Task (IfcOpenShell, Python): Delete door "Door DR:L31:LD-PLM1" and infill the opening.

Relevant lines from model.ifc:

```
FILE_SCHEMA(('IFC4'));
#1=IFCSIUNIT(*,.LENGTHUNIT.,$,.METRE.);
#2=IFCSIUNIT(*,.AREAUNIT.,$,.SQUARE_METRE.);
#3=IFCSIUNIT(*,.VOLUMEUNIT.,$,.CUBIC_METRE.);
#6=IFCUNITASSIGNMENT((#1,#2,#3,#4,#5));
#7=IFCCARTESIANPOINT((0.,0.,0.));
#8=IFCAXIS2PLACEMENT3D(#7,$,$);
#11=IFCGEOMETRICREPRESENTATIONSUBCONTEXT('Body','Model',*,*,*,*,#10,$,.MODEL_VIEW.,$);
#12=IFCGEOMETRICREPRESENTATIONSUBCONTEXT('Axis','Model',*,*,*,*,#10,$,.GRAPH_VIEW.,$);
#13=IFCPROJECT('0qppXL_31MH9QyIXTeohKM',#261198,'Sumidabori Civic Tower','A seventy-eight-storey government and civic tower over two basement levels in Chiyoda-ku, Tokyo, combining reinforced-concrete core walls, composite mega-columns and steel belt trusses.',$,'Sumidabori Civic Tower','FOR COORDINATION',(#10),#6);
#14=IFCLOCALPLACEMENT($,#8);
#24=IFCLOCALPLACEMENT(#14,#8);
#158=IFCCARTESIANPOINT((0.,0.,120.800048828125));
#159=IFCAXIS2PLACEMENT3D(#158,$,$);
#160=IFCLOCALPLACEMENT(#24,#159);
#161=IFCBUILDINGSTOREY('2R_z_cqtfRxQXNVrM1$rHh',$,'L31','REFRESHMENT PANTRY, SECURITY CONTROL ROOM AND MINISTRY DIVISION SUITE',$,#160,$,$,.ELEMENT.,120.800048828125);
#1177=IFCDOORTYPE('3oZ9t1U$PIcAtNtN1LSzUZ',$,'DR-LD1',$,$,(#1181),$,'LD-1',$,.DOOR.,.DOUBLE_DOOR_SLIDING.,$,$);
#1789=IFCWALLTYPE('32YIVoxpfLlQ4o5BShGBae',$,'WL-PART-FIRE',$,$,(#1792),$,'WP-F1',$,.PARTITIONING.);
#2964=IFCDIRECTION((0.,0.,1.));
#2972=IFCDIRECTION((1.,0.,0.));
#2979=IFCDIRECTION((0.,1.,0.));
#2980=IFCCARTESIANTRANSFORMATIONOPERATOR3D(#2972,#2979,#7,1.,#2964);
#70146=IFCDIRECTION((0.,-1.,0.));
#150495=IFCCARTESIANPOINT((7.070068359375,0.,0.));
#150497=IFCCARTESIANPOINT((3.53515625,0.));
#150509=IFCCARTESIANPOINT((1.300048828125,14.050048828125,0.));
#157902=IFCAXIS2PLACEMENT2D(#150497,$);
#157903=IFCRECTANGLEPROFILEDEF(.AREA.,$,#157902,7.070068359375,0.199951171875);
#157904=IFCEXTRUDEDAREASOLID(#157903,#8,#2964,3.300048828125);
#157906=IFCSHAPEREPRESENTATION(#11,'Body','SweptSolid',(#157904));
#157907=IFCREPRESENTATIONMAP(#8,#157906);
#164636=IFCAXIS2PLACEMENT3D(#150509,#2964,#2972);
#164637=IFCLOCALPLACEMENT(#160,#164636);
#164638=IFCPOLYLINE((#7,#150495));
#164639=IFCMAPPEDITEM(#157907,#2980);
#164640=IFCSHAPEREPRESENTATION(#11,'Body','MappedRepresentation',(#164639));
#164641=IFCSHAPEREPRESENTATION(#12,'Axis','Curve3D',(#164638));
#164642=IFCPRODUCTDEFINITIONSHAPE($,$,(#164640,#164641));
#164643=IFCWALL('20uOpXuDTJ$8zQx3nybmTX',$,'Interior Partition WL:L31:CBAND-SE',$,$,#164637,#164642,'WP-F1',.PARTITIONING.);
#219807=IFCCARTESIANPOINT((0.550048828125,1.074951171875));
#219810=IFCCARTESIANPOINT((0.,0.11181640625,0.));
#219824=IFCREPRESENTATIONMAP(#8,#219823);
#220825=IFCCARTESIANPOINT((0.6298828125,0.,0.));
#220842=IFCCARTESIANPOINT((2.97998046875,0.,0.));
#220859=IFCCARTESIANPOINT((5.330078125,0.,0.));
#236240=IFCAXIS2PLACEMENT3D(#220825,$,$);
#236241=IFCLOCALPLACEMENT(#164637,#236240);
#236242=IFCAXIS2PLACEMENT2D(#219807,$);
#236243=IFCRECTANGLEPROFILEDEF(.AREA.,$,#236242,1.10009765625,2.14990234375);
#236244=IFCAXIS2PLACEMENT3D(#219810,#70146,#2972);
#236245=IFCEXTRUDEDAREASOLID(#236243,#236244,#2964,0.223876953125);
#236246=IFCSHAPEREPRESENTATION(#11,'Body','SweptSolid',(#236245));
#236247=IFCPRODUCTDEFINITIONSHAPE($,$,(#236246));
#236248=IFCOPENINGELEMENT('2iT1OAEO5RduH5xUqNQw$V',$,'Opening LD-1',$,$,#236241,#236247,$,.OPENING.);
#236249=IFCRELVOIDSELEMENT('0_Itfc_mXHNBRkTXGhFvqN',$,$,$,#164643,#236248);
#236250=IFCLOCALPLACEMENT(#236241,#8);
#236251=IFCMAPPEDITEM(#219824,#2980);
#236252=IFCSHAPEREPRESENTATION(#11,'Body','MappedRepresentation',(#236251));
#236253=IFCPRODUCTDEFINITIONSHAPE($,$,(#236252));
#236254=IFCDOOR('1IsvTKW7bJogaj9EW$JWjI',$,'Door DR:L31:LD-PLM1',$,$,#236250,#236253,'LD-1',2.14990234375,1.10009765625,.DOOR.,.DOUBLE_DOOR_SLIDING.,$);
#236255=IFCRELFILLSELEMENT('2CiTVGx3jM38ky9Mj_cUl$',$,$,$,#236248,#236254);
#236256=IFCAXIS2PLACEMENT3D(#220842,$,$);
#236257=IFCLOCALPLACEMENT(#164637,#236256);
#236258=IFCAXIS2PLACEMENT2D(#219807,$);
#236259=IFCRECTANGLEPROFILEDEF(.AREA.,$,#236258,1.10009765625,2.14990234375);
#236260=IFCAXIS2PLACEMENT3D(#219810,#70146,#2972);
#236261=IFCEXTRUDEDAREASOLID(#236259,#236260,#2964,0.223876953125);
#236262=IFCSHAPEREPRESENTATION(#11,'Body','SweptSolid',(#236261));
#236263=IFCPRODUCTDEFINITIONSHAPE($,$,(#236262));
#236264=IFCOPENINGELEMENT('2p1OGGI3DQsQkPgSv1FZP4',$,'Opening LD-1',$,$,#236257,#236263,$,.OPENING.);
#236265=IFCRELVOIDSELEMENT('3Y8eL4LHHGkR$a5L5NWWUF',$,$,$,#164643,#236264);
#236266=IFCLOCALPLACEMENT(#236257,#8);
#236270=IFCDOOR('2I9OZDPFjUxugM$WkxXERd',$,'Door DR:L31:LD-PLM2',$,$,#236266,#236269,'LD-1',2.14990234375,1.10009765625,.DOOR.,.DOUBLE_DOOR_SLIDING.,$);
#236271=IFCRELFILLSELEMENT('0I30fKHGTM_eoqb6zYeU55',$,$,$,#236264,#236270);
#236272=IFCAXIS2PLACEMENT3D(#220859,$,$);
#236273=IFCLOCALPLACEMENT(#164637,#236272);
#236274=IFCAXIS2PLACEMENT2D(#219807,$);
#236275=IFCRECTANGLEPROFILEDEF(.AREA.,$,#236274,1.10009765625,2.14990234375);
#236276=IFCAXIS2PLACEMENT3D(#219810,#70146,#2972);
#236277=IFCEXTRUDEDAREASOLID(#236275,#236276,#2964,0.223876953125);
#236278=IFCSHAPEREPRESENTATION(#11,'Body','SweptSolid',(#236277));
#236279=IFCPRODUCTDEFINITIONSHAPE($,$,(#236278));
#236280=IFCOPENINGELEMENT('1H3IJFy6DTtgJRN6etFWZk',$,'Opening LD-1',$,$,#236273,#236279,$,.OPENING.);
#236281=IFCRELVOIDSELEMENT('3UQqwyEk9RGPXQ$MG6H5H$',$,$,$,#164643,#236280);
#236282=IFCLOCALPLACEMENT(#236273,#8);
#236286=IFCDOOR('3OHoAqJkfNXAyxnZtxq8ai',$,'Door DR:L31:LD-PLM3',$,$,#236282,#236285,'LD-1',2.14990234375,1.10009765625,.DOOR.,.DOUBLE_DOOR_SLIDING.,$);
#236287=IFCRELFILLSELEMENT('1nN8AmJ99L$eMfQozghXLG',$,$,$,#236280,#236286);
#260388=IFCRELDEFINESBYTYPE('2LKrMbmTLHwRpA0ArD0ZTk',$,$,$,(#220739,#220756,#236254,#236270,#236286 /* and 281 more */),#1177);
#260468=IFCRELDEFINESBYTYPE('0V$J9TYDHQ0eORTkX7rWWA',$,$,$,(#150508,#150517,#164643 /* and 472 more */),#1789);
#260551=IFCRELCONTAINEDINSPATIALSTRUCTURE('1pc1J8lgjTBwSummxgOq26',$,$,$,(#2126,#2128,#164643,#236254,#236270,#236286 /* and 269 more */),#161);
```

```python
import ifcopenshell
import ifcopenshell.api.feature
import ifcopenshell.api.root
import ifcopenshell.geom
import ifcopenshell.util.shape

model = ifcopenshell.open("model.ifc")
settings = ifcopenshell.geom.settings()


def volume(element):
    """Net volume in cubic metres, openings subtracted."""
    shape = ifcopenshell.geom.create_shape(settings, element)
    return ifcopenshell.util.shape.get_volume(shape.geometry)


door = model.by_id(236254)
opening = door.FillsVoids[0].RelatingOpeningElement
wall = opening.VoidsElements[0].RelatingBuildingElement
before = volume(wall)

ifcopenshell.api.root.remove_product(model, product=door)
ifcopenshell.api.feature.remove_feature(model, feature=opening)

after = volume(wall)

print(f"wall volume {before:.3f} -> {after:.3f} m3")

model.write("model_rev.ifc")
```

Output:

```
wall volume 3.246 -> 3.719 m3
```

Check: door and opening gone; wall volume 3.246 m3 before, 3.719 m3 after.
